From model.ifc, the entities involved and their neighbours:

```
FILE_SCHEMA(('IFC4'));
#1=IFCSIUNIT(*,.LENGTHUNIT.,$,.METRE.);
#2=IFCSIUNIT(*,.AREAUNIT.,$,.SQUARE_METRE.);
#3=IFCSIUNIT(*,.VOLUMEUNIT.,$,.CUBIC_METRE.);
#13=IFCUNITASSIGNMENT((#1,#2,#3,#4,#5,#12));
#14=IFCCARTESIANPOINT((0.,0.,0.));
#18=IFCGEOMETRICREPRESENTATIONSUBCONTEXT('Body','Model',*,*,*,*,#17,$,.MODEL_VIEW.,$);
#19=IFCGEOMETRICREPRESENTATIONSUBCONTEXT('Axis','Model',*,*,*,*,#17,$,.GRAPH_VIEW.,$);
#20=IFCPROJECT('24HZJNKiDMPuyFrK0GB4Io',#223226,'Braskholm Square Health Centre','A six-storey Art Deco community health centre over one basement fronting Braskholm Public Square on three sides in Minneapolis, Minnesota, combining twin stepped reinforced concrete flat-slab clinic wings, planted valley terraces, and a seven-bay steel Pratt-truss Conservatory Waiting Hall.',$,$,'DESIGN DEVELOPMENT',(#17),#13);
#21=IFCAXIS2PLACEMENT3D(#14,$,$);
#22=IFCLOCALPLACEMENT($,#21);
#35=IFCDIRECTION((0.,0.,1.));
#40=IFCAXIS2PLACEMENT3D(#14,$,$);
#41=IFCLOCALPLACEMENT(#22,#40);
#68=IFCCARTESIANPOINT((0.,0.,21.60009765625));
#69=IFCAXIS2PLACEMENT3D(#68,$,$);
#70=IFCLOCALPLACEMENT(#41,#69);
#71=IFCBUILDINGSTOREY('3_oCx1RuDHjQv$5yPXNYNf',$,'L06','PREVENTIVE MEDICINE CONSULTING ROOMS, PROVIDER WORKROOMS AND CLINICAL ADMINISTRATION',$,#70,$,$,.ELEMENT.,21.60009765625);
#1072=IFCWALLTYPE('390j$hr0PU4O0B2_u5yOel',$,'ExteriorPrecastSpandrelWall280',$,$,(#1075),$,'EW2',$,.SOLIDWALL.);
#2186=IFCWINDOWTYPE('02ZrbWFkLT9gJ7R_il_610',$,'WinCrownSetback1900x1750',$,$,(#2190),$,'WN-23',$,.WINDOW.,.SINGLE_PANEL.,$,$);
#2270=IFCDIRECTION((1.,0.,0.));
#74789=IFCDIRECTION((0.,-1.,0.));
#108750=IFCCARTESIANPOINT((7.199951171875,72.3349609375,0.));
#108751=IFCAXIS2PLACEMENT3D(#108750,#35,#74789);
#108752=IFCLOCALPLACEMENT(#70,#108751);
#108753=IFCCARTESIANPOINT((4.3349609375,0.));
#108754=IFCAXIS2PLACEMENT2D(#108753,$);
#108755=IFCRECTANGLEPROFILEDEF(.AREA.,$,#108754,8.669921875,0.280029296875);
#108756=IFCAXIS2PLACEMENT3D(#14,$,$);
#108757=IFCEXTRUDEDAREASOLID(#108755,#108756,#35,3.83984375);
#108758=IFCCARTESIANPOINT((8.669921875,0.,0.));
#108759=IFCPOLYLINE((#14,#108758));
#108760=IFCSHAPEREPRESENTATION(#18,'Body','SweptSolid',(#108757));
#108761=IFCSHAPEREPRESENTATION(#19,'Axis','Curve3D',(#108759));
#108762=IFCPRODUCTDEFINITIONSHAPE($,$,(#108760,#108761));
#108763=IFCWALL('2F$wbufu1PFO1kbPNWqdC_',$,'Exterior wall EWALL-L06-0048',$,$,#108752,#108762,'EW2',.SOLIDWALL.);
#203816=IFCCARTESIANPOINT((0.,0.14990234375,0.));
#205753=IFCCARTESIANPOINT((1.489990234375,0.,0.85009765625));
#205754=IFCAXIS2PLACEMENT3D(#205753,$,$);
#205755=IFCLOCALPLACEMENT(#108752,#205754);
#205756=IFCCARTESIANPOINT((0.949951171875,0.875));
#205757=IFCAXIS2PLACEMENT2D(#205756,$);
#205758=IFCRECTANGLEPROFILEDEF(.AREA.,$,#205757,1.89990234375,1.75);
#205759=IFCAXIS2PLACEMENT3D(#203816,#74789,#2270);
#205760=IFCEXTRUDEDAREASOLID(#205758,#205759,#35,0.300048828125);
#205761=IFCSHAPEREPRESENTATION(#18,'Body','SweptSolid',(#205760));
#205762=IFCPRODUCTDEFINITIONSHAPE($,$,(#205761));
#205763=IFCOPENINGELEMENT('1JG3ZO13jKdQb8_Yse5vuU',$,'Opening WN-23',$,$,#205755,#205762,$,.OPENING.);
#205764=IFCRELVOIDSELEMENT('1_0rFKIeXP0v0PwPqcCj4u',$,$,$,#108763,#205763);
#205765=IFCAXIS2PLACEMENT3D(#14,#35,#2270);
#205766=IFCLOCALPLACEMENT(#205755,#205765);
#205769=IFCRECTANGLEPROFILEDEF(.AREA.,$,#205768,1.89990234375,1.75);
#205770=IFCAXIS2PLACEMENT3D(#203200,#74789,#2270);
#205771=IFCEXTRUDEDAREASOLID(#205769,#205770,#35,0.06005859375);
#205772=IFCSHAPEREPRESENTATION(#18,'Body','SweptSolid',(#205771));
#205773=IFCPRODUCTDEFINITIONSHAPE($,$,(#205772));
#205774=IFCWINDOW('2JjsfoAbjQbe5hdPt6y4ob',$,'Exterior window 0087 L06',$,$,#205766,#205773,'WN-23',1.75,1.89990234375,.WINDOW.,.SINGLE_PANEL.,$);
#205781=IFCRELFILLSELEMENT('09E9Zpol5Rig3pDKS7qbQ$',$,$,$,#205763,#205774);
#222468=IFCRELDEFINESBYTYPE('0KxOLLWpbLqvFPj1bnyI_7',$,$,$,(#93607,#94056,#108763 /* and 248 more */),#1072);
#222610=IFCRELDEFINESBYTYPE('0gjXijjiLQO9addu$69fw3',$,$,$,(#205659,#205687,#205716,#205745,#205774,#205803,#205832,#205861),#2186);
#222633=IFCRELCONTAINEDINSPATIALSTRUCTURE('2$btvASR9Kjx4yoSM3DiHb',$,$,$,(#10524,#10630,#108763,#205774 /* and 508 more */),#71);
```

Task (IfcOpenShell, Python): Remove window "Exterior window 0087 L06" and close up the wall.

```python
import ifcopenshell
import ifcopenshell.api.feature
import ifcopenshell.api.root
import ifcopenshell.geom
import ifcopenshell.util.shape

model = ifcopenshell.open("model.ifc")
settings = ifcopenshell.geom.settings()


def volume(element):
    """Net volume in cubic metres, openings subtracted."""
    shape = ifcopenshell.geom.create_shape(settings, element)
    return ifcopenshell.util.shape.get_volume(shape.geometry)


window = model.by_guid("2JjsfoAbjQbe5hdPt6y4ob")
opening = window.FillsVoids[0].RelatingOpeningElement
wall = opening.VoidsElements[0].RelatingBuildingElement
before = volume(wall)

ifcopenshell.api.root.remove_product(model, product=window)
ifcopenshell.api.feature.remove_feature(model, feature=opening)

after = volume(wall)

print(f"wall volume {before:.3f} -> {after:.3f} m3")

model.write("model-out.ifc")
```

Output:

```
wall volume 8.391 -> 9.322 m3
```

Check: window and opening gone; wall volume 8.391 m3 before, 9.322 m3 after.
